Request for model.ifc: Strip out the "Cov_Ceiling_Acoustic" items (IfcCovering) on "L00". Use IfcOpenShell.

First a look at what the model holds.

```python
import ifcopenshell
import ifcopenshell.util.element

model = ifcopenshell.open("model.ifc")
print(model.schema)
storey = next(s for s in model.by_type("IfcBuildingStorey") if s.Name == "L00")
coverings = [e for e in ifcopenshell.util.element.get_decomposition(storey) if e.is_a("IfcCovering")]
seen = {}
for e in coverings:
    element_type = ifcopenshell.util.element.get_type(e)
    name = element_type.Name if element_type not in (None, e) else None
    seen[name] = seen.get(name, 0) + 1
for name, count in sorted(seen.items(), key=str):
    print(count, "x", name)
```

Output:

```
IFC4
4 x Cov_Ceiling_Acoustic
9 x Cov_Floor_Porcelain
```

```python
import ifcopenshell
import ifcopenshell.api.root
import ifcopenshell.util.element

model = ifcopenshell.open("model.ifc")

storey = next(s for s in model.by_type("IfcBuildingStorey") if s.Name == "L00")
coverings = [e for e in ifcopenshell.util.element.get_decomposition(storey) if e.is_a("IfcCovering")]
targets = [e for e in coverings if (t := ifcopenshell.util.element.get_type(e)) not in (None, e) and t.Name == "Cov_Ceiling_Acoustic"]

for e in targets:
    ifcopenshell.api.root.remove_product(model, product=e)
print(len(targets), "removed")

model.write("model_updated.ifc")
```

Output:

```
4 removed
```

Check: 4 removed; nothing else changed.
